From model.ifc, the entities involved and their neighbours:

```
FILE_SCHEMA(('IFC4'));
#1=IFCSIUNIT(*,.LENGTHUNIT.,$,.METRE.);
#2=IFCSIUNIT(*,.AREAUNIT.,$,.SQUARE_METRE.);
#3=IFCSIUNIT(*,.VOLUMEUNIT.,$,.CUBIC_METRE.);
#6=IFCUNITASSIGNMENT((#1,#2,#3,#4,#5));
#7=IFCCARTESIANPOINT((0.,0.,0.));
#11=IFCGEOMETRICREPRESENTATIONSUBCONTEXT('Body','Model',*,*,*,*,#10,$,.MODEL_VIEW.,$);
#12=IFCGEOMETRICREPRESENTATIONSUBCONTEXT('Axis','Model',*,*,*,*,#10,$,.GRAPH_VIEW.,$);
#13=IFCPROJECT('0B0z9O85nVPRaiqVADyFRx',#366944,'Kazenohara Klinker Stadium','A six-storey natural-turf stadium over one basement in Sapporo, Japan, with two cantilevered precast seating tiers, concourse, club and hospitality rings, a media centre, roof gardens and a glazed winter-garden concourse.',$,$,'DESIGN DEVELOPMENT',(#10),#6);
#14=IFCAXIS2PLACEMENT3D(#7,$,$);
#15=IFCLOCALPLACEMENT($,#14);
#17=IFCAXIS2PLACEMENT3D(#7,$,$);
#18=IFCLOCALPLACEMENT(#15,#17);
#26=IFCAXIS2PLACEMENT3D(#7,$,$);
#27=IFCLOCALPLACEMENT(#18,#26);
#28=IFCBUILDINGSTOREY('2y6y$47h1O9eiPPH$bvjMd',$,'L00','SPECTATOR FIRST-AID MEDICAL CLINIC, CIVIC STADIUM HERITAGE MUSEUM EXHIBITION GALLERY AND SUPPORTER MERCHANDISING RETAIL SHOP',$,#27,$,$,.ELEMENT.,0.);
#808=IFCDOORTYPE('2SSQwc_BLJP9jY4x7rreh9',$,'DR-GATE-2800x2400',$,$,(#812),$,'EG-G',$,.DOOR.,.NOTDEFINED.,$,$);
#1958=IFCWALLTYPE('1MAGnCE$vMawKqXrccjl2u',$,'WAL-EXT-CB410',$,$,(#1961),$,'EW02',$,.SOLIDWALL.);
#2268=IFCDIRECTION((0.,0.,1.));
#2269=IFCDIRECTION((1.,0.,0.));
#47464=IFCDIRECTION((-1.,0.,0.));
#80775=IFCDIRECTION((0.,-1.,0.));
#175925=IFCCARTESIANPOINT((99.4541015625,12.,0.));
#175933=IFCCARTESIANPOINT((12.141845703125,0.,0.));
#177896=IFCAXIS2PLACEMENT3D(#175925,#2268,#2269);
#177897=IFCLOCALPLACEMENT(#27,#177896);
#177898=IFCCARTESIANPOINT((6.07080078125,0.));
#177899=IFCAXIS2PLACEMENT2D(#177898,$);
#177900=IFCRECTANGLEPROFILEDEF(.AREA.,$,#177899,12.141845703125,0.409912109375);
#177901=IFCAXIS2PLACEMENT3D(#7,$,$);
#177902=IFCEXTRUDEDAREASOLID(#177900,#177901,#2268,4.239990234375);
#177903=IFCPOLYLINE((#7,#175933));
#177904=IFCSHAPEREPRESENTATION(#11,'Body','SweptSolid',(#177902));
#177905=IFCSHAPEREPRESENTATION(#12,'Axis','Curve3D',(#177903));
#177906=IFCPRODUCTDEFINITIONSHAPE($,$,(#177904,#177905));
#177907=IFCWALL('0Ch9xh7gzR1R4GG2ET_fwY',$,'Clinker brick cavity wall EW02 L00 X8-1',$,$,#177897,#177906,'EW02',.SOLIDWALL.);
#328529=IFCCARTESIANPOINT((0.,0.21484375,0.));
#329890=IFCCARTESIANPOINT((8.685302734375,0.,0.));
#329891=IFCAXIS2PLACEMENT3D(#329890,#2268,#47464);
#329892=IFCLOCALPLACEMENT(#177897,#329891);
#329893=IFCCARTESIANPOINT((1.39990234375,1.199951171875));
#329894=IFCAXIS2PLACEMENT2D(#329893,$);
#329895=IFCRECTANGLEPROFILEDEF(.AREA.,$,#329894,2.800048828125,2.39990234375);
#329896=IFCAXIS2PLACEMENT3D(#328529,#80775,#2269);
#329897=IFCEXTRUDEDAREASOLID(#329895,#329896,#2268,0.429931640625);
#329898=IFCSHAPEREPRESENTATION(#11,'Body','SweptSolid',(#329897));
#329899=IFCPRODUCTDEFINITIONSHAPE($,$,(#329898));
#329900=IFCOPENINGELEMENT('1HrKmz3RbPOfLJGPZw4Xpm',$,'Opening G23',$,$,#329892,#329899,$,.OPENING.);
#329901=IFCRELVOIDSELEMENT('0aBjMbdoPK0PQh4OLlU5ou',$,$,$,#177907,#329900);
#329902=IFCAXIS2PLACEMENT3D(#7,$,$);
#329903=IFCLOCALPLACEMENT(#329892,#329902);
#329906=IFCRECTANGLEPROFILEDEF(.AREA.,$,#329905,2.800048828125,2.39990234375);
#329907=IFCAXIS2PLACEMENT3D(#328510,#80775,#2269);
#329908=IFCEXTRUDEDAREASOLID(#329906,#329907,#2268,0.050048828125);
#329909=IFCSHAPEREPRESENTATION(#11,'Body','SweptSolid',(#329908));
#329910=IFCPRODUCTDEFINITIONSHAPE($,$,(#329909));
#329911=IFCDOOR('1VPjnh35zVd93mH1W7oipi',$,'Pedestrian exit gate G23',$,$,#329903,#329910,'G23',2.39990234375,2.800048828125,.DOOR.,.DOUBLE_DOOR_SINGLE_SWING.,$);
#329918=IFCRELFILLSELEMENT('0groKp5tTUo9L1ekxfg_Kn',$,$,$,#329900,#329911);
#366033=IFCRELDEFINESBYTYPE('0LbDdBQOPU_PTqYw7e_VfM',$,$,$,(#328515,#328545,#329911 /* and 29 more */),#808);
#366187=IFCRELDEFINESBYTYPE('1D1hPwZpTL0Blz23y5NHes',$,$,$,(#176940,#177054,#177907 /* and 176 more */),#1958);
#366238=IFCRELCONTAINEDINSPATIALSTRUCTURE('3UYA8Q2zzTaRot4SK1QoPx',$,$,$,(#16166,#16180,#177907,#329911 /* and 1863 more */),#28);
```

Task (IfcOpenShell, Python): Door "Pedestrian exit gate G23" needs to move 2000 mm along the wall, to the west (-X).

```python
import ifcopenshell
import ifcopenshell.api.geometry
import ifcopenshell.util.placement
import ifcopenshell.util.unit

model = ifcopenshell.open("model.ifc")
unit_scale = ifcopenshell.util.unit.calculate_unit_scale(model)

door = model.by_guid("1VPjnh35zVd93mH1W7oipi")
opening = door.FillsVoids[0].RelatingOpeningElement
wall = opening.VoidsElements[0].RelatingBuildingElement

wall_matrix = ifcopenshell.util.placement.get_local_placement(wall.ObjectPlacement)
shift = wall_matrix[:3, 0] * -2 / unit_scale
before = ifcopenshell.util.placement.get_local_placement(door.ObjectPlacement)[:3, 3].copy()

# The door is placed relative to its opening, so it follows when the opening moves.
matrix = ifcopenshell.util.placement.get_local_placement(opening.ObjectPlacement)
matrix[:3, 3] += shift
ifcopenshell.api.geometry.edit_object_placement(
    model, product=opening, matrix=matrix, is_si=False, should_transform_children=True
)

after = ifcopenshell.util.placement.get_local_placement(door.ObjectPlacement)[:3, 3]
print("door moved by", (after - before).round(3) + 0.0)

model.write("model_updated.ifc")
```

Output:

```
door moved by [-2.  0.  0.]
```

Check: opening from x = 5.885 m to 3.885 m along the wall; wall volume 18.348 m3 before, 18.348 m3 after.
